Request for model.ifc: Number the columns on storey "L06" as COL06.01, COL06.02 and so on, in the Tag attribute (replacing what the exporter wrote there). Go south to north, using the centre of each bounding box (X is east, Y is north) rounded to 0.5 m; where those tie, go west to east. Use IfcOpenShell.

First a look at what the model holds.

```python
import ifcopenshell
import ifcopenshell.util.element
import ifcopenshell.util.placement

model = ifcopenshell.open("model.ifc")
print(model.schema)
storey = next(s for s in model.by_type("IfcBuildingStorey") if s.Name == "L06")
columns = [e for e in ifcopenshell.util.element.get_decomposition(storey) if e.is_a("IfcColumn")]
for e in sorted(columns, key=lambda e: e.id()):
    origin = ifcopenshell.util.placement.get_local_placement(e.ObjectPlacement)[:3, 3]
    print(e.id(), e.Tag, e.Name, origin.round(2) + 0.0, sep=" | ")
```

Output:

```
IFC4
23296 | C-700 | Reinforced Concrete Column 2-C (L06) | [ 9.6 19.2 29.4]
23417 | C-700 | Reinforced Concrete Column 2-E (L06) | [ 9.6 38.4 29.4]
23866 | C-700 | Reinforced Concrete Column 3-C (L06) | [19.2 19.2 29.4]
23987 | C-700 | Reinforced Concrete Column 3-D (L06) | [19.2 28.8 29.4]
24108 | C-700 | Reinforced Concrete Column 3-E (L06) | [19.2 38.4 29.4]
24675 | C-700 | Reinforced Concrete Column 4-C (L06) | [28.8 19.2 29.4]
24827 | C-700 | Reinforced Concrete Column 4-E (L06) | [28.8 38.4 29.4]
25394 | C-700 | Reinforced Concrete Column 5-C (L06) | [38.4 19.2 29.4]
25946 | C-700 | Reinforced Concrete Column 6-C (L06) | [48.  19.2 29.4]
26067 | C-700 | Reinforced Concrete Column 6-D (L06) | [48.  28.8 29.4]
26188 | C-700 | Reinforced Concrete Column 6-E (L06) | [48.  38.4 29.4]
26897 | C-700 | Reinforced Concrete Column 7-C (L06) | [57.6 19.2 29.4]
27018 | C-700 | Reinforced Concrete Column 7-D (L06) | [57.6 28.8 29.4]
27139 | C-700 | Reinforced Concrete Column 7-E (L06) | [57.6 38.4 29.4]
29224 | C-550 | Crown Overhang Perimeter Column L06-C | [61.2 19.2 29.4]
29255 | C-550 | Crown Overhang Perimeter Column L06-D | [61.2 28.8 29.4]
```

```python
import ifcopenshell
import ifcopenshell.geom
import ifcopenshell.util.element
import ifcopenshell.util.shape

model = ifcopenshell.open("model.ifc")
settings = ifcopenshell.geom.settings()
settings.set("use-world-coords", True)


def centre(element):
    shape = ifcopenshell.geom.create_shape(settings, element)
    return ifcopenshell.util.shape.get_bbox_centroid(shape.geometry)


storey = next(s for s in model.by_type("IfcBuildingStorey") if s.Name == "L06")
columns = [e for e in ifcopenshell.util.element.get_decomposition(storey) if e.is_a("IfcColumn")]

# Insertion points can sit at a corner or the storey origin, so sort by the geometry (in metres).
centres = {e: centre(e) for e in columns}
columns.sort(key=lambda e: (round(centres[e][1] / 0.5), centres[e][0]))

for i, e in enumerate(columns, start=1):
    number = f"COL06.{i:02d}"
    e.Tag = number
    print(e.id(), number)

model.write("model_updated.ifc")
```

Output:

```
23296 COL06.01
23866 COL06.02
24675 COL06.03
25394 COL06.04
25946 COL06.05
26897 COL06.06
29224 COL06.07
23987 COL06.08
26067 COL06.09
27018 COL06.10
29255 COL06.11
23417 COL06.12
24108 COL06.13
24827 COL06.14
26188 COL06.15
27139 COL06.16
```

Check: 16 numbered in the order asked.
